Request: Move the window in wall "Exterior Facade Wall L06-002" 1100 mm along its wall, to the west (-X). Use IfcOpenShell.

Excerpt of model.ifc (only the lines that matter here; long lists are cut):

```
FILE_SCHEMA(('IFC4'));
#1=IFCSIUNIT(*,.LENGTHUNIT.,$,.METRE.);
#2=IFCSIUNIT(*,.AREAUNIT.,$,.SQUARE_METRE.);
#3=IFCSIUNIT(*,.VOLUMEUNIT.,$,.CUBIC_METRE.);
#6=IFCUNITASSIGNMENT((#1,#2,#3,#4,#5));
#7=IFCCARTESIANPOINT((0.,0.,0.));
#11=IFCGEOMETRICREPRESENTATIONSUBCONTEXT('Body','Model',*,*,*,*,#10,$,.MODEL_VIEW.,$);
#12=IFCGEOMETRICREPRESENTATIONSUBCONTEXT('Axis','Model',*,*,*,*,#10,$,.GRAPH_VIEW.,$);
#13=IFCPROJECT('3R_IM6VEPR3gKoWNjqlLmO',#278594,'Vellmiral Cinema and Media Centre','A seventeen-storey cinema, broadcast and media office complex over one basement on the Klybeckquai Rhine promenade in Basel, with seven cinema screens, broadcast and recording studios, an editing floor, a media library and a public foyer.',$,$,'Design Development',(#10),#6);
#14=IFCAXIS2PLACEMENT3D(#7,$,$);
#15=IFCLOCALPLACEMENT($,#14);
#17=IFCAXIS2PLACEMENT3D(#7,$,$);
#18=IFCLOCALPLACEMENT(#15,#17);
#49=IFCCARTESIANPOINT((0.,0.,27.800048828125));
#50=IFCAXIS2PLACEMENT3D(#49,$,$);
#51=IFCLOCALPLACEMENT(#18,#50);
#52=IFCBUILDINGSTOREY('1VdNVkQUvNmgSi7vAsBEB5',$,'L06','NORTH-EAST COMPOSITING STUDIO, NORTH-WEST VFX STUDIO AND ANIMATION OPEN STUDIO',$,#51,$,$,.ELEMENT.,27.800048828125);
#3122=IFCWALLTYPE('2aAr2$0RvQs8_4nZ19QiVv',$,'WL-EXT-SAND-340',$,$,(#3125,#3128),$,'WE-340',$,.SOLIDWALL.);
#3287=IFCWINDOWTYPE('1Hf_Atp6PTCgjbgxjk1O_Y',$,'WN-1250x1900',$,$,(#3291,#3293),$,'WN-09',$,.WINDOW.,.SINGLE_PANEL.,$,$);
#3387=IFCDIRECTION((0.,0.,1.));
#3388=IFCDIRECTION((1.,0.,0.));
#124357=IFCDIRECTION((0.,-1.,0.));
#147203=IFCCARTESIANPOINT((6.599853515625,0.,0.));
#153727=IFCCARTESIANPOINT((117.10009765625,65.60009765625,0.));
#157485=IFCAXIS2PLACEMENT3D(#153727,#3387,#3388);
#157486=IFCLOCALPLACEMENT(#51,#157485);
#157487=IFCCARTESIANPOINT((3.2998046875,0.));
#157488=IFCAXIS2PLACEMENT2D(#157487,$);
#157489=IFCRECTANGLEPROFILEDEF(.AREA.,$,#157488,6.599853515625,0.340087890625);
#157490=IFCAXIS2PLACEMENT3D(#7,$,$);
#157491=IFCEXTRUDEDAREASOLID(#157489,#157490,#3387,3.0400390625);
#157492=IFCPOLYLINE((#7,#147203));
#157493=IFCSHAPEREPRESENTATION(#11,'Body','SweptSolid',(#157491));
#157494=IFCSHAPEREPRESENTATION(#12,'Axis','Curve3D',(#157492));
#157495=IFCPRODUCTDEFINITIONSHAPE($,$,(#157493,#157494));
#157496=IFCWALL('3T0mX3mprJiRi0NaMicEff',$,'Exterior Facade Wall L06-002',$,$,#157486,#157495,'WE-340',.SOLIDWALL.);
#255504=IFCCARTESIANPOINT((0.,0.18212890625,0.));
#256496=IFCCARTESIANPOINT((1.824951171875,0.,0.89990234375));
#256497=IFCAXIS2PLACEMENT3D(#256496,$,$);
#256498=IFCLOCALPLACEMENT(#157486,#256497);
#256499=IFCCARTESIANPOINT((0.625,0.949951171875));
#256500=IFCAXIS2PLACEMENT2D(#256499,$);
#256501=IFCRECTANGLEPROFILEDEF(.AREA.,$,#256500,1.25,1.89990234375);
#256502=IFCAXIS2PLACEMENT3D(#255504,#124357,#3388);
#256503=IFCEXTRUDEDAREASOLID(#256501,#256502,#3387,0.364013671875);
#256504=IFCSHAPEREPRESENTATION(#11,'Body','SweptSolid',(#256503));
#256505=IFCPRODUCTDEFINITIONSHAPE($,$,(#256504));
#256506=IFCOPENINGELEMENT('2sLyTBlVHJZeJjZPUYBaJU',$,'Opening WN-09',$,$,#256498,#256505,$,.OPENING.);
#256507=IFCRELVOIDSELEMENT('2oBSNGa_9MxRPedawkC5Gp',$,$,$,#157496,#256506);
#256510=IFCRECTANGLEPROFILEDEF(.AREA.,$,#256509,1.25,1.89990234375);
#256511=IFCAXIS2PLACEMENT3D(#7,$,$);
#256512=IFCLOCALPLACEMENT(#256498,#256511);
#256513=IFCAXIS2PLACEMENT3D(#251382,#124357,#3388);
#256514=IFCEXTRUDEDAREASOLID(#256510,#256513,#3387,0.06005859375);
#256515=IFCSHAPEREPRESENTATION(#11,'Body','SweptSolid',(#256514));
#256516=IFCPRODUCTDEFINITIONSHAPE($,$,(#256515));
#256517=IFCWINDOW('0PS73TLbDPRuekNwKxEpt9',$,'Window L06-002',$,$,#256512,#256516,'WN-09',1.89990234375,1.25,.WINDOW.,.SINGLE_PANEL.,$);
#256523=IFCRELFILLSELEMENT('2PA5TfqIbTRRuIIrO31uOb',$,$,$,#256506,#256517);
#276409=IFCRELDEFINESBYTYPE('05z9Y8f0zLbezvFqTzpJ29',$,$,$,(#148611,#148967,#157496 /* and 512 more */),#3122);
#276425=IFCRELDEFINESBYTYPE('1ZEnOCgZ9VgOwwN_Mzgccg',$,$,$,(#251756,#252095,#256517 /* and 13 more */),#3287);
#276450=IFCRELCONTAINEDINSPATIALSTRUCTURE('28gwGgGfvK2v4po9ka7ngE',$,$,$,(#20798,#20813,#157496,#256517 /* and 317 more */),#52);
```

```python
import ifcopenshell
import ifcopenshell.api.geometry
import ifcopenshell.util.placement

model = ifcopenshell.open("model.ifc")

window = model.by_id(256517)
opening = window.FillsVoids[0].RelatingOpeningElement
wall = opening.VoidsElements[0].RelatingBuildingElement

wall_matrix = ifcopenshell.util.placement.get_local_placement(wall.ObjectPlacement)
shift = wall_matrix[:3, 0] * -1.1
before = ifcopenshell.util.placement.get_local_placement(window.ObjectPlacement)[:3, 3].copy()

# The window is placed relative to its opening, so it follows when the opening moves.
matrix = ifcopenshell.util.placement.get_local_placement(opening.ObjectPlacement)
matrix[:3, 3] += shift
ifcopenshell.api.geometry.edit_object_placement(
    model, product=opening, matrix=matrix, is_si=False, should_transform_children=True
)

after = ifcopenshell.util.placement.get_local_placement(window.ObjectPlacement)[:3, 3]
print("window moved by", (after - before).round(3) + 0.0)

model.write("model_v2.ifc")
```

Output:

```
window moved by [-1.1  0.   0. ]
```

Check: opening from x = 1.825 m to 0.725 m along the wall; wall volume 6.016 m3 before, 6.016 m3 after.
